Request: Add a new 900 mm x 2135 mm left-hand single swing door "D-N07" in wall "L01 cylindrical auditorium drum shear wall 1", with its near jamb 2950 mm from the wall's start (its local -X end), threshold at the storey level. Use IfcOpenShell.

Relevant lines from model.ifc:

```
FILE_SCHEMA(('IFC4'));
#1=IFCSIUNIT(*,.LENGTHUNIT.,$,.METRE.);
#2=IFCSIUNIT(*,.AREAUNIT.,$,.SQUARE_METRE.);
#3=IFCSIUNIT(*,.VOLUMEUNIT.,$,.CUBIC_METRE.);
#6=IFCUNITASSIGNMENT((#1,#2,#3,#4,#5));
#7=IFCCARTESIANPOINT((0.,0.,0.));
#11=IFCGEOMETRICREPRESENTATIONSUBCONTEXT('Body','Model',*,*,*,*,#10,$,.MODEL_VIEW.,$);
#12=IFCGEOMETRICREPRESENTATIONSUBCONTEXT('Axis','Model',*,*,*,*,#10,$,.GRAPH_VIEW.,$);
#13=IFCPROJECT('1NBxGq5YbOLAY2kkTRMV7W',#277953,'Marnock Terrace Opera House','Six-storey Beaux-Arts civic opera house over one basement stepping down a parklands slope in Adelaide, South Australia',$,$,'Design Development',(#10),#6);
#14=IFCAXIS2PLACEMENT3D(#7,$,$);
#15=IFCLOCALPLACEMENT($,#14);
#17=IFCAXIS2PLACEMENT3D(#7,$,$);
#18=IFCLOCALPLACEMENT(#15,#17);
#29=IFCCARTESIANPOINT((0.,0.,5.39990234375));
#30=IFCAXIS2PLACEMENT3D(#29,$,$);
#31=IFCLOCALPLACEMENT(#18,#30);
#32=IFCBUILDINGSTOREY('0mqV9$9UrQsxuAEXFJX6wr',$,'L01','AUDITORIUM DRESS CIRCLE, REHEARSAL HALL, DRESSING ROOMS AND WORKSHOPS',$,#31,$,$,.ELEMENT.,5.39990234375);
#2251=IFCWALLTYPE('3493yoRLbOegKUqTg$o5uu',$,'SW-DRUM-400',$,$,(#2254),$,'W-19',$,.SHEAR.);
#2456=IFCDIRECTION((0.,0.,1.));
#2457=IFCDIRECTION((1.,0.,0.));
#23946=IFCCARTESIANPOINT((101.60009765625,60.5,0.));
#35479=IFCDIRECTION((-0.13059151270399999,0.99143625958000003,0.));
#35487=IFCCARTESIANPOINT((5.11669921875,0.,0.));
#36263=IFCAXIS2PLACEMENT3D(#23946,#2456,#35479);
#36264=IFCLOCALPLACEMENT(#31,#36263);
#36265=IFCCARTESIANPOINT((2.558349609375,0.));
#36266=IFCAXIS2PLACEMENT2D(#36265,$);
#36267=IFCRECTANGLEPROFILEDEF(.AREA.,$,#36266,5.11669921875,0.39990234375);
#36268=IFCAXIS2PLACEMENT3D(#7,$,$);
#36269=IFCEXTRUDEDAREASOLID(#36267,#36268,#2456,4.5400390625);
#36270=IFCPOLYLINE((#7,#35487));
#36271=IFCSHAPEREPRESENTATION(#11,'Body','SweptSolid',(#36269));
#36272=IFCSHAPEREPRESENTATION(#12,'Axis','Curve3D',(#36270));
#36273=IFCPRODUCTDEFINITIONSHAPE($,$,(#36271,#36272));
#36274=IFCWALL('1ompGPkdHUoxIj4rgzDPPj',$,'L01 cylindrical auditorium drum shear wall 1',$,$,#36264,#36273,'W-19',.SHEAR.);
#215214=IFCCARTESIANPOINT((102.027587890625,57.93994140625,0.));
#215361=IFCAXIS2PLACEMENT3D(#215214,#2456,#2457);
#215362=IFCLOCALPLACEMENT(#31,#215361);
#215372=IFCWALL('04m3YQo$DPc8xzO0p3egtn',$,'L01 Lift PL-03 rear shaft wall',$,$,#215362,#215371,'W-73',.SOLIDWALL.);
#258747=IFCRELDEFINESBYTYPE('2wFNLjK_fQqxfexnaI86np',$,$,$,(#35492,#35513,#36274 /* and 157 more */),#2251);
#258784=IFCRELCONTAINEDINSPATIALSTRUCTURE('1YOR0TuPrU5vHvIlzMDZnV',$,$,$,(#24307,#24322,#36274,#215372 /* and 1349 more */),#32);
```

```python
import numpy as np
import ifcopenshell
import ifcopenshell.api.feature
import ifcopenshell.api.geometry
import ifcopenshell.api.root
import ifcopenshell.api.spatial
import ifcopenshell.geom
import ifcopenshell.util.element
import ifcopenshell.util.placement
import ifcopenshell.util.representation
import ifcopenshell.util.shape
import ifcopenshell.util.unit

model = ifcopenshell.open("model.ifc")
unit_scale = ifcopenshell.util.unit.calculate_unit_scale(model)
settings = ifcopenshell.geom.settings()


def volume(element):
    """Net volume in cubic metres, openings subtracted."""
    shape = ifcopenshell.geom.create_shape(settings, element)
    return ifcopenshell.util.shape.get_volume(shape.geometry)


wall = model.by_id(36274)
storey = ifcopenshell.util.element.get_container(wall, ifc_class="IfcBuildingStorey")
context = ifcopenshell.util.representation.get_context(model, "Model", "Body", "MODEL_VIEW")
before = volume(wall)

width, height, from_end, sill = 0.9, 2.135, 2.95, 0.0  # metres

# The wall runs along its own X axis, and the end named is its -X end.
wall_shape = ifcopenshell.geom.create_shape(settings, wall)
x, y, z = ifcopenshell.util.shape.get_vertices(wall_shape.geometry).T
start = x.min() + from_end
face, thickness = float(y.min()), float(y.max() - y.min())
wall_matrix = ifcopenshell.util.placement.get_local_placement(wall.ObjectPlacement)
level = ifcopenshell.util.placement.get_local_placement(storey.ObjectPlacement)[2, 3]


def in_wall(x, y):
    """Placement at x, y metres in the wall's axes, at sill height."""
    matrix = wall_matrix.copy()
    matrix[:, 3] = wall_matrix @ np.array([x / unit_scale, y / unit_scale, 0.0, 1.0])
    matrix[2, 3] = level + sill / unit_scale
    return matrix


# Opening: a box that overshoots both wall faces by 50 mm.
opening = ifcopenshell.api.root.create_entity(model, ifc_class="IfcOpeningElement", predefined_type="OPENING")
box = ifcopenshell.api.geometry.add_wall_representation(
    model, context=context, length=width, height=height, thickness=thickness + 0.1
)
ifcopenshell.api.geometry.assign_representation(model, product=opening, representation=box)
ifcopenshell.api.geometry.edit_object_placement(model, product=opening, matrix=in_wall(start, face - 0.05), is_si=False)
ifcopenshell.api.feature.add_feature(model, feature=opening, element=wall)

door = ifcopenshell.api.root.create_entity(model, ifc_class="IfcDoor", name="D-N07", predefined_type="DOOR")
door.OverallWidth, door.OverallHeight = width / unit_scale, height / unit_scale
door.OperationType = "SINGLE_SWING_LEFT"
body = ifcopenshell.api.geometry.add_door_representation(
    model,
    context=context,
    overall_width=door.OverallWidth,
    overall_height=door.OverallHeight,
    operation_type="SINGLE_SWING_LEFT",
    lining_properties={"LiningDepth": thickness / unit_scale, "ThresholdDepth": thickness / unit_scale},
)
ifcopenshell.api.geometry.assign_representation(model, product=door, representation=body)
ifcopenshell.api.spatial.assign_container(model, products=[door], relating_structure=storey)
ifcopenshell.api.feature.add_filling(model, opening=opening, element=door)

# The lining spans the wall, so the door starts at the wall face.
ifcopenshell.api.geometry.edit_object_placement(model, product=door, matrix=in_wall(start, face), is_si=False)

after = volume(wall)

print(f"wall volume {before:.3f} -> {after:.3f} m3")

model.write("model_updated.ifc")
```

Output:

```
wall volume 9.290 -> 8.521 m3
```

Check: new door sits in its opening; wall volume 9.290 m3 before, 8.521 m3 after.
